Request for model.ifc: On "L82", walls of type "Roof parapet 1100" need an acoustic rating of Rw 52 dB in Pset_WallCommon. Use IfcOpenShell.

First a look at what the model holds.

```python
import ifcopenshell
import ifcopenshell.util.element

model = ifcopenshell.open("model.ifc")
print(model.schema)
storey = next(s for s in model.by_type("IfcBuildingStorey") if s.Name == "L82")
walls = [e for e in ifcopenshell.util.element.get_decomposition(storey) if e.is_a("IfcWall")]
seen = {}
for e in walls:
    element_type = ifcopenshell.util.element.get_type(e)
    key = (element_type.Name if element_type != e and element_type else None, ifcopenshell.util.element.get_pset(e, "Pset_WallCommon", "AcousticRating"))
    seen[key] = seen.get(key, 0) + 1
for (name, value), count in sorted(seen.items(), key=str):
    print(count, "x", name, "|", value)
```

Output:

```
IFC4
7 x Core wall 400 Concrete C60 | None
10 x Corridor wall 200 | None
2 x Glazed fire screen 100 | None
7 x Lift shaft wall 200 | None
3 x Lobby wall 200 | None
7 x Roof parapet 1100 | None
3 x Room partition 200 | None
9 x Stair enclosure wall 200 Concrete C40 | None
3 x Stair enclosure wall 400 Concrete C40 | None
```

```python
import ifcopenshell
import ifcopenshell.api.pset
import ifcopenshell.util.element

model = ifcopenshell.open("model.ifc")

storey = next(s for s in model.by_type("IfcBuildingStorey") if s.Name == "L82")
walls = [e for e in ifcopenshell.util.element.get_decomposition(storey) if e.is_a("IfcWall")]

count = 0
for e in walls:
    element_type = ifcopenshell.util.element.get_type(e)
    if element_type in (None, e) or element_type.Name != "Roof parapet 1100":
        continue
    found = ifcopenshell.util.element.get_pset(e, "Pset_WallCommon", should_inherit=False)
    if found:
        pset = model.by_id(found["id"])
        if len(ifcopenshell.util.element.get_elements_by_pset(pset)) > 1:
            pset = ifcopenshell.api.pset.unshare_pset(model, products=[e], pset=pset)[0]
    else:
        pset = ifcopenshell.api.pset.add_pset(model, product=e, name="Pset_WallCommon")
    ifcopenshell.api.pset.edit_pset(model, pset=pset, properties={"AcousticRating": "Rw 52 dB"})
    count += 1

print(count, "walls updated")

model.write("model-out.ifc")
```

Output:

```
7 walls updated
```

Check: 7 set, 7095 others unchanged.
